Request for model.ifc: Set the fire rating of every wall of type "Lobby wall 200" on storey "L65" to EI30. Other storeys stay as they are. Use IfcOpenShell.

First a look at what the model holds.

```python
import ifcopenshell
import ifcopenshell.util.element

model = ifcopenshell.open("model.ifc")
print(model.schema)
storey = next(s for s in model.by_type("IfcBuildingStorey") if s.Name == "L65")
walls = [e for e in ifcopenshell.util.element.get_decomposition(storey) if e.is_a("IfcWall")]
seen = {}
for e in walls:
    element_type = ifcopenshell.util.element.get_type(e)
    key = (element_type.Name if element_type != e and element_type else None, ifcopenshell.util.element.get_pset(e, "Pset_WallCommon", "FireRating"))
    seen[key] = seen.get(key, 0) + 1
for (name, value), count in sorted(seen.items(), key=str):
    print(count, "x", name, "|", value)
```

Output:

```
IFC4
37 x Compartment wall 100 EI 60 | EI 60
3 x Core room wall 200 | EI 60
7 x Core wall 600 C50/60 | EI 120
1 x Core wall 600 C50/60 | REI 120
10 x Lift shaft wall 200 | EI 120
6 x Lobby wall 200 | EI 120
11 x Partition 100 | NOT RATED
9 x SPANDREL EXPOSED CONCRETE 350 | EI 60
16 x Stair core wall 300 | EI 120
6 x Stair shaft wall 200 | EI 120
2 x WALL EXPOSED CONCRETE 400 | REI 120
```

```python
import ifcopenshell
import ifcopenshell.api.pset
import ifcopenshell.util.element

model = ifcopenshell.open("model.ifc")

storey = next(s for s in model.by_type("IfcBuildingStorey") if s.Name == "L65")
walls = [e for e in ifcopenshell.util.element.get_decomposition(storey) if e.is_a("IfcWall")]

count = 0
for e in walls:
    element_type = ifcopenshell.util.element.get_type(e)
    if element_type in (None, e) or element_type.Name != "Lobby wall 200":
        continue
    found = ifcopenshell.util.element.get_pset(e, "Pset_WallCommon", should_inherit=False)
    if found:
        pset = model.by_id(found["id"])
        if len(ifcopenshell.util.element.get_elements_by_pset(pset)) > 1:
            pset = ifcopenshell.api.pset.unshare_pset(model, products=[e], pset=pset)[0]
    else:
        pset = ifcopenshell.api.pset.add_pset(model, product=e, name="Pset_WallCommon")
    ifcopenshell.api.pset.edit_pset(model, pset=pset, properties={"FireRating": "EI30"})
    count += 1

print(count, "walls updated")

model.write("model_v2.ifc")
```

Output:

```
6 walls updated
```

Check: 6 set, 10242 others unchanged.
